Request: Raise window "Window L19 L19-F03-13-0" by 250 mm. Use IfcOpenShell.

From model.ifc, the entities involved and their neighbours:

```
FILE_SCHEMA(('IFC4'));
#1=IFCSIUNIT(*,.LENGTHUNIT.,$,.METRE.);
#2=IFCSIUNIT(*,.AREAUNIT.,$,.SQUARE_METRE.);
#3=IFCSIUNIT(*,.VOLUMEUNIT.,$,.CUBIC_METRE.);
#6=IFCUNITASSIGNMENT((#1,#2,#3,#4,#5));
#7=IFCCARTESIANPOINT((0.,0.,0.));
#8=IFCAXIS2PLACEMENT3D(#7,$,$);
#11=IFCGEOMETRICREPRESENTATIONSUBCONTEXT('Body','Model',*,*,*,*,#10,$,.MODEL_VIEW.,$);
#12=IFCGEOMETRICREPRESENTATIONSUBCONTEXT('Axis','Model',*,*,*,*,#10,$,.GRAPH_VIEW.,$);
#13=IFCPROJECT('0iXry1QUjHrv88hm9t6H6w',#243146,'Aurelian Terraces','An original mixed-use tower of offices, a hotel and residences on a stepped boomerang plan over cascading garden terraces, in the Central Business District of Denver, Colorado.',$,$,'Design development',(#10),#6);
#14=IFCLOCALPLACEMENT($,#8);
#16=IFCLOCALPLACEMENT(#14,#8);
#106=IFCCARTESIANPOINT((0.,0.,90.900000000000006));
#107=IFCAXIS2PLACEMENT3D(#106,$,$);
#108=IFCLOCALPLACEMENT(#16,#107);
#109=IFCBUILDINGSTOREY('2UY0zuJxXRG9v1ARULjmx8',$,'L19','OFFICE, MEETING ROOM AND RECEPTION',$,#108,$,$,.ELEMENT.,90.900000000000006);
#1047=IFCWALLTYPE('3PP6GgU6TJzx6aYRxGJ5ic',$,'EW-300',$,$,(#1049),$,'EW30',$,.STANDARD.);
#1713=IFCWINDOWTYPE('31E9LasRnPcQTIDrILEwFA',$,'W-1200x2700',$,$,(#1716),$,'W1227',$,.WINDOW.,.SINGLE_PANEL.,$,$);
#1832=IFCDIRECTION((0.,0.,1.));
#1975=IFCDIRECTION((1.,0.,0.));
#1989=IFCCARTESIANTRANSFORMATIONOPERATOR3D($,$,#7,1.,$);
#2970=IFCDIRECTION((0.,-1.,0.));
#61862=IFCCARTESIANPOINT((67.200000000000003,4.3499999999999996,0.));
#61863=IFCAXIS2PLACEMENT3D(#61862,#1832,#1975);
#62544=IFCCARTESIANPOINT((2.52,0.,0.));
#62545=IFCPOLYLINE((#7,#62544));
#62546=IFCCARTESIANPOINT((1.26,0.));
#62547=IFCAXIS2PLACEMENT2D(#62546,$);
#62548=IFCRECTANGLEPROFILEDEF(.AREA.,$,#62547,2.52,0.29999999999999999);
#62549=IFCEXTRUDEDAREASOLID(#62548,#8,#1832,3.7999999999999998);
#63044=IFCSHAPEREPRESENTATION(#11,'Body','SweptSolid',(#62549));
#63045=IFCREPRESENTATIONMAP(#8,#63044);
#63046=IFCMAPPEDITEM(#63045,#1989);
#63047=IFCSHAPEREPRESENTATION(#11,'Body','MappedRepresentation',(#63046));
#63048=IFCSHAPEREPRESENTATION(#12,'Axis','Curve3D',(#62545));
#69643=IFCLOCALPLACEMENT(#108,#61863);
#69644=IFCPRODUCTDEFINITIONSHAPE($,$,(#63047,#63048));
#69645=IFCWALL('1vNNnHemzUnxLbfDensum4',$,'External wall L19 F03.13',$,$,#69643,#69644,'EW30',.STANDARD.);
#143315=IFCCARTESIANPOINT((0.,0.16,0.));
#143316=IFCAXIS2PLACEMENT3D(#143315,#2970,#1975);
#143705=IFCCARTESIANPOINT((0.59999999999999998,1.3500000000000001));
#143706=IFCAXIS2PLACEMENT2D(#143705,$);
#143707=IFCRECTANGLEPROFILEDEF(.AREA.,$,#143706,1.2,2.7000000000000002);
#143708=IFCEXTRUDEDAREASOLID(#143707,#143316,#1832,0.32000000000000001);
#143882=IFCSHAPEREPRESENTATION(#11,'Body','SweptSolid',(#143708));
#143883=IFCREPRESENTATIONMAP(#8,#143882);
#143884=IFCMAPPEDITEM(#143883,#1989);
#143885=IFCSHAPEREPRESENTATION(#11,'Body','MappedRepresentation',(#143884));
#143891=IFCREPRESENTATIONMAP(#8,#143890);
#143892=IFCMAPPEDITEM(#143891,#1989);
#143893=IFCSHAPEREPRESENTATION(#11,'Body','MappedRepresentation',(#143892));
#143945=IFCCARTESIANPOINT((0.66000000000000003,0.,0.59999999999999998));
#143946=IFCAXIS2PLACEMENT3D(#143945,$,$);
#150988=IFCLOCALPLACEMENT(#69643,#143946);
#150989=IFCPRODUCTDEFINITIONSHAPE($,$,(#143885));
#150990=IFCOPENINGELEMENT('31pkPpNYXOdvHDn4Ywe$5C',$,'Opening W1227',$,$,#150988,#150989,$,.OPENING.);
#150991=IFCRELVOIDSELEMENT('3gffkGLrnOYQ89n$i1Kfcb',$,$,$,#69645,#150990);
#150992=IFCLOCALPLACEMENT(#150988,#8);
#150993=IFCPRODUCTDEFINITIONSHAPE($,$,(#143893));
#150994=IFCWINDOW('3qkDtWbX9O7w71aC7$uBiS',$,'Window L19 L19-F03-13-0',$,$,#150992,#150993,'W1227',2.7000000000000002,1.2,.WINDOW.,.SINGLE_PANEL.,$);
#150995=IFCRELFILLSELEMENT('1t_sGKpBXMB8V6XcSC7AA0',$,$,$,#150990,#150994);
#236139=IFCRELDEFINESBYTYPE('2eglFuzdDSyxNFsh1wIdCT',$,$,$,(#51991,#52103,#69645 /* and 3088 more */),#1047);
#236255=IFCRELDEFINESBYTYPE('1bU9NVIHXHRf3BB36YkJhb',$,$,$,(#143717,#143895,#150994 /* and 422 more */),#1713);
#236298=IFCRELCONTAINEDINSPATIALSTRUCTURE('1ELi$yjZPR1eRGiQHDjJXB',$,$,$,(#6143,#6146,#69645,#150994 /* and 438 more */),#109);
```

```python
import numpy as np
import ifcopenshell
import ifcopenshell.api.geometry
import ifcopenshell.util.placement
import ifcopenshell.util.unit

model = ifcopenshell.open("model.ifc")
unit_scale = ifcopenshell.util.unit.calculate_unit_scale(model)

window = model.by_guid("3qkDtWbX9O7w71aC7$uBiS")
opening = window.FillsVoids[0].RelatingOpeningElement
dz = 0.25 / unit_scale

shift = np.array([0.0, 0.0, dz])
# The window is placed relative to its opening, so it follows when the opening moves.
matrix = ifcopenshell.util.placement.get_local_placement(opening.ObjectPlacement)
matrix[:3, 3] += shift
ifcopenshell.api.geometry.edit_object_placement(
    model, product=opening, matrix=matrix, is_si=False, should_transform_children=True
)

print(f"moved by {dz * unit_scale:+.3f} m")

model.write("model_rev.ifc")
```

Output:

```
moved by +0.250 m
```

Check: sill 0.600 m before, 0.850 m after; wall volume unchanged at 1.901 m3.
